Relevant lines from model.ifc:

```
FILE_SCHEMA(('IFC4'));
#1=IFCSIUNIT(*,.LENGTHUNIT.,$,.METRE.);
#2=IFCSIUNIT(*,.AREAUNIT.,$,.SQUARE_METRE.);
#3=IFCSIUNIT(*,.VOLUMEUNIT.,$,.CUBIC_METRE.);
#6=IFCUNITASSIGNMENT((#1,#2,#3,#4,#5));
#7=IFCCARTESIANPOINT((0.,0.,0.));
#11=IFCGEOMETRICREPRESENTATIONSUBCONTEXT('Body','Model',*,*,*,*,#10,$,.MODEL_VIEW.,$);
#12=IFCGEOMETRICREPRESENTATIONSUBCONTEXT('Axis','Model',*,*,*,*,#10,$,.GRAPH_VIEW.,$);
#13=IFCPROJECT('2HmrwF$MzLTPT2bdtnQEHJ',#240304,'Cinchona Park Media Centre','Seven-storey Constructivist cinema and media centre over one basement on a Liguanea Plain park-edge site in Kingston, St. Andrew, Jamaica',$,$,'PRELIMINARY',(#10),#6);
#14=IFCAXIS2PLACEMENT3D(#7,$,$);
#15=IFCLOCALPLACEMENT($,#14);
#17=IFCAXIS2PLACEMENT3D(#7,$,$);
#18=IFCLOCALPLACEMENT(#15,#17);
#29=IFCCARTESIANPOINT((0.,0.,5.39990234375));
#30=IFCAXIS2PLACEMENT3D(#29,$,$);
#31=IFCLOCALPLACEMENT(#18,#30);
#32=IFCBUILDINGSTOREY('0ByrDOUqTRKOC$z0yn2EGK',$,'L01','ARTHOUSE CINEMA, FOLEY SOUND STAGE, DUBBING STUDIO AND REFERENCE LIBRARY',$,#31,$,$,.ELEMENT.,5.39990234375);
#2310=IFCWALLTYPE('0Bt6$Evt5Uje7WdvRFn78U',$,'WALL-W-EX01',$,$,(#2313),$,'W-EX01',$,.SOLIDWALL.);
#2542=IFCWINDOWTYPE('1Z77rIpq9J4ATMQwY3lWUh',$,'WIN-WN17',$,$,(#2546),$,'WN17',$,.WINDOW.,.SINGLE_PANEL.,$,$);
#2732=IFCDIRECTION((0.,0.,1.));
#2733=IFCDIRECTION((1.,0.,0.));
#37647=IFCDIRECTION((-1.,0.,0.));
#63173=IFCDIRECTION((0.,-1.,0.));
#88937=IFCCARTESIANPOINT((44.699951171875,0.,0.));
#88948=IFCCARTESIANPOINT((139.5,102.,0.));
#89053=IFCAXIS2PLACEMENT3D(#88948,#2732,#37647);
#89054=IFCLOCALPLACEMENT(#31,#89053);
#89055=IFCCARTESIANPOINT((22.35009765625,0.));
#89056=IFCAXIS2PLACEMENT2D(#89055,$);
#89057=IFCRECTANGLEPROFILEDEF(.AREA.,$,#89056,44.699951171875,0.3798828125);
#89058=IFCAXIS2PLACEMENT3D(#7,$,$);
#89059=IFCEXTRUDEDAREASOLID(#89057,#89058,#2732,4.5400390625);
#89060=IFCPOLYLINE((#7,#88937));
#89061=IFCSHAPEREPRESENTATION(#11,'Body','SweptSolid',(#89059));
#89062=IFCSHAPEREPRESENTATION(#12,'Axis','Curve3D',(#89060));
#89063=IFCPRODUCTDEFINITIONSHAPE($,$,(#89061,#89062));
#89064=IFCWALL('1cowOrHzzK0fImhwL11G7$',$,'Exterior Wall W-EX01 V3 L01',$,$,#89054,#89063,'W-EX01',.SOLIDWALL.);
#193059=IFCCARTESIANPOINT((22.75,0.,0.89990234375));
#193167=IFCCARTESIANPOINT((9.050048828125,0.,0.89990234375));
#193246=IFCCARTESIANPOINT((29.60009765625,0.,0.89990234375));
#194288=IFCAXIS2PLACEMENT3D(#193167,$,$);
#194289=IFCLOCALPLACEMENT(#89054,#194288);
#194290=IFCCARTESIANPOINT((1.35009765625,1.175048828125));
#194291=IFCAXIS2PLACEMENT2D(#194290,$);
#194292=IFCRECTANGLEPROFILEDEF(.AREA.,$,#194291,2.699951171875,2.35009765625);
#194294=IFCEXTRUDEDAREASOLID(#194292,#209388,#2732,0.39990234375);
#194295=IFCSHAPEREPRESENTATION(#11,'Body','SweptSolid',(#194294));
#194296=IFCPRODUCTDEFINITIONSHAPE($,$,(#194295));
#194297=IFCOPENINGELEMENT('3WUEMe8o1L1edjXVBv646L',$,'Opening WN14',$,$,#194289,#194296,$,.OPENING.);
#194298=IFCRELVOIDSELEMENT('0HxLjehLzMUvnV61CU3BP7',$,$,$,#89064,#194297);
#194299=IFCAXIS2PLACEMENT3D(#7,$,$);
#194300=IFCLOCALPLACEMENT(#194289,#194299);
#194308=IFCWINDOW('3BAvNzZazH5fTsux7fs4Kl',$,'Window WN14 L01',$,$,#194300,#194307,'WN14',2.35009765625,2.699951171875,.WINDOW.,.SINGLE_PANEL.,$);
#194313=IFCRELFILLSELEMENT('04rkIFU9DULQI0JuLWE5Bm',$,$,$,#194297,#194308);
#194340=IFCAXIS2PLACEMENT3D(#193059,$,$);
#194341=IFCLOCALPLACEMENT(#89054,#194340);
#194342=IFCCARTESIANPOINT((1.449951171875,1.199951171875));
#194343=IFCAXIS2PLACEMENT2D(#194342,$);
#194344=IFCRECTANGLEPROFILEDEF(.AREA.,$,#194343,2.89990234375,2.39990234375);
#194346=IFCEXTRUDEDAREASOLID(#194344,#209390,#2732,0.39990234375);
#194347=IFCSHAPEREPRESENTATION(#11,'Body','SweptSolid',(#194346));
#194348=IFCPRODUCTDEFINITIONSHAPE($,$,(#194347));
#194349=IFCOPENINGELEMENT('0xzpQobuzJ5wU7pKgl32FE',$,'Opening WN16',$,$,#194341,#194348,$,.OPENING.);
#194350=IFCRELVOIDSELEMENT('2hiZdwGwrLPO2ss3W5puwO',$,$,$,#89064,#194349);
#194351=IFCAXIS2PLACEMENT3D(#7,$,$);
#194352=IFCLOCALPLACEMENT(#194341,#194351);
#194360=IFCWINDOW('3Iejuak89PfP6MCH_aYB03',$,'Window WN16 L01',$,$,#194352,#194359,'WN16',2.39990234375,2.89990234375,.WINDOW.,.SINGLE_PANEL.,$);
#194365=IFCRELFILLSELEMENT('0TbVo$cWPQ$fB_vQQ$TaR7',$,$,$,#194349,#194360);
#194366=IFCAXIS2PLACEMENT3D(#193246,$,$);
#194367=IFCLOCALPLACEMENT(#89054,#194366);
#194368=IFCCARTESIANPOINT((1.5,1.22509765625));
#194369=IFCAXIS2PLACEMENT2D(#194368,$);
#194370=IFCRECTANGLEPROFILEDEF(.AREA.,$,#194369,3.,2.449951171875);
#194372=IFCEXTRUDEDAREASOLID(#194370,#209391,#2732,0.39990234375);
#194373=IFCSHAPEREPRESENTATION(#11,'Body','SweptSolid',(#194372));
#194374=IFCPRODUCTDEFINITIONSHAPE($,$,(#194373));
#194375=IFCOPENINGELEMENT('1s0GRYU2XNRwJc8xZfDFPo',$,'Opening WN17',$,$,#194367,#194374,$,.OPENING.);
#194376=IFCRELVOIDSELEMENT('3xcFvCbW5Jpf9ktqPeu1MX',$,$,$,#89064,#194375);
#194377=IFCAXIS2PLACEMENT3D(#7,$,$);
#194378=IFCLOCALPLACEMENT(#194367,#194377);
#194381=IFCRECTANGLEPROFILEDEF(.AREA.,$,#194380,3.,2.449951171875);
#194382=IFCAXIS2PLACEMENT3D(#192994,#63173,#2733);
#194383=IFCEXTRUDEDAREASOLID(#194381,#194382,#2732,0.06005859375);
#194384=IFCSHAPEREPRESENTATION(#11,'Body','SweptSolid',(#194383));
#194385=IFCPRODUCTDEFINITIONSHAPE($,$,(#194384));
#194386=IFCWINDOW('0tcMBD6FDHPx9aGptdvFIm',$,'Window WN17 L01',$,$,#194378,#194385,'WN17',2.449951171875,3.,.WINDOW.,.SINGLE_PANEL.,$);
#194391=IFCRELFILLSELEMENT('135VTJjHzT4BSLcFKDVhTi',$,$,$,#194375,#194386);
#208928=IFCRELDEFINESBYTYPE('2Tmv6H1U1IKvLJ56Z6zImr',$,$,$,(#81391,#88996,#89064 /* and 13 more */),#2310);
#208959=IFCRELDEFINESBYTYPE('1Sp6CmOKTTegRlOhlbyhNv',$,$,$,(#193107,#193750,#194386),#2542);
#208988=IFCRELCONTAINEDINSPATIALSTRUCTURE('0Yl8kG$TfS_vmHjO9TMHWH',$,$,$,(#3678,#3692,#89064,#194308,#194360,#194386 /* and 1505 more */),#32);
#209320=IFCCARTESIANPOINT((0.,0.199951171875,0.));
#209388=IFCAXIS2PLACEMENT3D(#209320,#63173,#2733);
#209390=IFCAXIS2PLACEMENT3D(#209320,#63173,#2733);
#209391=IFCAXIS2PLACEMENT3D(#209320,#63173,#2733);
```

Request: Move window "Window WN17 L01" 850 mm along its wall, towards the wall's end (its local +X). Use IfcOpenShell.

```python
import ifcopenshell
import ifcopenshell.api.geometry
import ifcopenshell.util.placement
import ifcopenshell.util.unit

model = ifcopenshell.open("model.ifc")
unit_scale = ifcopenshell.util.unit.calculate_unit_scale(model)

window = model.by_guid("0tcMBD6FDHPx9aGptdvFIm")
opening = window.FillsVoids[0].RelatingOpeningElement
wall = opening.VoidsElements[0].RelatingBuildingElement

wall_matrix = ifcopenshell.util.placement.get_local_placement(wall.ObjectPlacement)
shift = wall_matrix[:3, 0] * 0.85 / unit_scale
before = ifcopenshell.util.placement.get_local_placement(window.ObjectPlacement)[:3, 3].copy()

# The window is placed relative to its opening, so it follows when the opening moves.
matrix = ifcopenshell.util.placement.get_local_placement(opening.ObjectPlacement)
matrix[:3, 3] += shift
ifcopenshell.api.geometry.edit_object_placement(
    model, product=opening, matrix=matrix, is_si=False, should_transform_children=True
)

after = ifcopenshell.util.placement.get_local_placement(window.ObjectPlacement)[:3, 3]
print("window moved by", (after - before).round(3) + 0.0)

model.write("model_updated.ifc")
```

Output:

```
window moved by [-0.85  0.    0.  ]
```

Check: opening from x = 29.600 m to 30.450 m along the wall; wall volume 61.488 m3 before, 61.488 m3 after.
